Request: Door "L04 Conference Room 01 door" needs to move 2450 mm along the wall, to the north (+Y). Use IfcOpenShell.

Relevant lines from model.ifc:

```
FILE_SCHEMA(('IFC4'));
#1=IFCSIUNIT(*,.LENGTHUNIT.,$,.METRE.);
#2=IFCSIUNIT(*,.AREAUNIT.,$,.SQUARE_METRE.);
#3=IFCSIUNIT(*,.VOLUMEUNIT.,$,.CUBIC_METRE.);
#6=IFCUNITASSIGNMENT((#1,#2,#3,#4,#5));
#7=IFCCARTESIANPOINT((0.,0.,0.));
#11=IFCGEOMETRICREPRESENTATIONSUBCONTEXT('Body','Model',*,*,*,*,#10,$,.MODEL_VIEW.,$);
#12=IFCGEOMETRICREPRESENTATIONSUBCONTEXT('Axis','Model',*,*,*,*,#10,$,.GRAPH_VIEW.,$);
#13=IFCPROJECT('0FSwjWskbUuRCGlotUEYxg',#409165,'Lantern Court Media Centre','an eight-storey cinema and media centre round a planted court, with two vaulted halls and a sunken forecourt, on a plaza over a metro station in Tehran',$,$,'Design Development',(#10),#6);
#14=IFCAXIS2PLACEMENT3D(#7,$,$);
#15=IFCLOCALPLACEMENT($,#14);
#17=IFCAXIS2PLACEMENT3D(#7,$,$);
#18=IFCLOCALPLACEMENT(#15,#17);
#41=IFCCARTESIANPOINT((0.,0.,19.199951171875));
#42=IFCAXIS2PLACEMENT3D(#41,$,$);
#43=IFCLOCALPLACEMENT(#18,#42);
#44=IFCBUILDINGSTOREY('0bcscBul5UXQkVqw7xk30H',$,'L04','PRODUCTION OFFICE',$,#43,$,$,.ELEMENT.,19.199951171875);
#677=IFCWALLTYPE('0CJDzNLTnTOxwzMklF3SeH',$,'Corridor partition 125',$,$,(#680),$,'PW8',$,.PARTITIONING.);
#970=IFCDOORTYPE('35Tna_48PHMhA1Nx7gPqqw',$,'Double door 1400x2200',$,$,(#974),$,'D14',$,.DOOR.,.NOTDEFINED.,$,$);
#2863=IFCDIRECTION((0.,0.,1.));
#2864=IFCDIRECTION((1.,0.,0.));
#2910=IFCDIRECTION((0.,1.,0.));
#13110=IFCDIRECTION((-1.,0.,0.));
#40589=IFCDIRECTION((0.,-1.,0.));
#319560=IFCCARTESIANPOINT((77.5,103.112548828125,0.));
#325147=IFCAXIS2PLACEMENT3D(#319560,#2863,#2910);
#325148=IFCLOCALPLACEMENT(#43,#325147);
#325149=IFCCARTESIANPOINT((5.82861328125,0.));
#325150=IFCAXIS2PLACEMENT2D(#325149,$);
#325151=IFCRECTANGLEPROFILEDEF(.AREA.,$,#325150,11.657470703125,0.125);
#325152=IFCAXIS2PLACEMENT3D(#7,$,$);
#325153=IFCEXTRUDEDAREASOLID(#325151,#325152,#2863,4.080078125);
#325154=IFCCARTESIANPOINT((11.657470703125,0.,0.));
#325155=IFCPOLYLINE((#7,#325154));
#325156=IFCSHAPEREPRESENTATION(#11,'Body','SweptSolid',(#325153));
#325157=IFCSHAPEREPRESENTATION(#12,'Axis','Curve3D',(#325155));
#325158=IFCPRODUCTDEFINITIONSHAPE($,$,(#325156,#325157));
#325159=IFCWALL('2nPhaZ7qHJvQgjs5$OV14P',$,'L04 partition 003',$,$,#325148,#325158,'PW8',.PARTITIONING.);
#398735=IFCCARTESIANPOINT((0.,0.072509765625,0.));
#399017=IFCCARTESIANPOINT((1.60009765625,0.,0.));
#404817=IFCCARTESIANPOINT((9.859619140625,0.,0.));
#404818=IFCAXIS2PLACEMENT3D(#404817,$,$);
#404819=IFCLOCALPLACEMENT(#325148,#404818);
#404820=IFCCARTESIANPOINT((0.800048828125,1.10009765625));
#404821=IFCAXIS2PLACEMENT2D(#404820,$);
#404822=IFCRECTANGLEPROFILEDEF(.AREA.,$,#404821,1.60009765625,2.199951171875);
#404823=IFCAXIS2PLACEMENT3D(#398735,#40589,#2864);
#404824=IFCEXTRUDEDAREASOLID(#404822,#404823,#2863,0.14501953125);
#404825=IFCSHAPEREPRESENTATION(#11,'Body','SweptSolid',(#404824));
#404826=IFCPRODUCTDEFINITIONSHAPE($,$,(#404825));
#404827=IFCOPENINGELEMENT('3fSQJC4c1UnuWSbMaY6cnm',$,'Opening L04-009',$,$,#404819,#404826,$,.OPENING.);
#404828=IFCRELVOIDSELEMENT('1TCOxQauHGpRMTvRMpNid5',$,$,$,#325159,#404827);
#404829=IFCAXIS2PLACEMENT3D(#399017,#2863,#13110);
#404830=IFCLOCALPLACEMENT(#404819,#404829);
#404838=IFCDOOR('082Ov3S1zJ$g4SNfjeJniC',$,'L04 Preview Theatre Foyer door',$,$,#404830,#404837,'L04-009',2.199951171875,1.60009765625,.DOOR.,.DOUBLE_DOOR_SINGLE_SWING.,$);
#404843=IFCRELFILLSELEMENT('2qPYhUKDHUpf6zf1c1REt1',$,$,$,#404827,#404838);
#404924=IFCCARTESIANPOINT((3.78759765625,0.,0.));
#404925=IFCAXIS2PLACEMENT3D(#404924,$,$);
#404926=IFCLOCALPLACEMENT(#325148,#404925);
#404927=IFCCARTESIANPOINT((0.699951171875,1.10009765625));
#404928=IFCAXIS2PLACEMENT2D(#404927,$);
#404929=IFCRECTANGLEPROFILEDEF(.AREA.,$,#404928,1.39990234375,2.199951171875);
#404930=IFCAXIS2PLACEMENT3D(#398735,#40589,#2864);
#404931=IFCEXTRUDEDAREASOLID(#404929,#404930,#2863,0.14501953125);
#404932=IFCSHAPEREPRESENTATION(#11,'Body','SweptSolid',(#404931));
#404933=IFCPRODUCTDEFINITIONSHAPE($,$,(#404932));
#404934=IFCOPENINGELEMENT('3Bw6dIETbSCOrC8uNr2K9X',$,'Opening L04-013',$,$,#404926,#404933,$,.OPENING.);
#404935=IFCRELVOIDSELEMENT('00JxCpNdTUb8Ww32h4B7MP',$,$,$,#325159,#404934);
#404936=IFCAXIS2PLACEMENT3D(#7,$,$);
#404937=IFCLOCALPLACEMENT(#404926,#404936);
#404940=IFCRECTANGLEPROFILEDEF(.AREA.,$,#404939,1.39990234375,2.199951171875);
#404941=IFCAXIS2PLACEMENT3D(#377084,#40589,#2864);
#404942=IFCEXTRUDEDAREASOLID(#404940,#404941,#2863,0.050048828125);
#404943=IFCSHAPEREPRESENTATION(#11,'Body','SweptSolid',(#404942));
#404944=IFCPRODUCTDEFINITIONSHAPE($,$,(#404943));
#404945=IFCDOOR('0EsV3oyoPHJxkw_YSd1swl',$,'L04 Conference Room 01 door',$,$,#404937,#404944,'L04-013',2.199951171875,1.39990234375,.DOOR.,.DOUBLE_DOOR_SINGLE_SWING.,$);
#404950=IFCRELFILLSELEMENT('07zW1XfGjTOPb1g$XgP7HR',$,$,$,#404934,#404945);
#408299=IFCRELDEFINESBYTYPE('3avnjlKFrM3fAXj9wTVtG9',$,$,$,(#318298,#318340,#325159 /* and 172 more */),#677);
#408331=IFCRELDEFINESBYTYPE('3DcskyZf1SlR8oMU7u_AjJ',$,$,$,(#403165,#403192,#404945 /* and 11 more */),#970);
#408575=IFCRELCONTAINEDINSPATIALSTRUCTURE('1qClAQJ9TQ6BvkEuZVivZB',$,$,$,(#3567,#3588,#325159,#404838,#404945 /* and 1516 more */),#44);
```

```python
import ifcopenshell
import ifcopenshell.api.geometry
import ifcopenshell.util.placement

model = ifcopenshell.open("model.ifc")

door = model.by_id(404945)
opening = door.FillsVoids[0].RelatingOpeningElement
wall = opening.VoidsElements[0].RelatingBuildingElement

wall_matrix = ifcopenshell.util.placement.get_local_placement(wall.ObjectPlacement)
shift = wall_matrix[:3, 0] * 2.45
before = ifcopenshell.util.placement.get_local_placement(door.ObjectPlacement)[:3, 3].copy()

# The door is placed relative to its opening, so it follows when the opening moves.
matrix = ifcopenshell.util.placement.get_local_placement(opening.ObjectPlacement)
matrix[:3, 3] += shift
ifcopenshell.api.geometry.edit_object_placement(
    model, product=opening, matrix=matrix, is_si=False, should_transform_children=True
)

after = ifcopenshell.util.placement.get_local_placement(door.ObjectPlacement)[:3, 3]
print("door moved by", (after - before).round(3) + 0.0)

model.write("model_updated.ifc")
```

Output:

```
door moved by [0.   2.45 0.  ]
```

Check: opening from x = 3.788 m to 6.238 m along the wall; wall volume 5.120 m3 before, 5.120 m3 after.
